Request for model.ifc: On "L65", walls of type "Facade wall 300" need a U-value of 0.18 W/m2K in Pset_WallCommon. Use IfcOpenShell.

First a look at what the model holds.

```python
import ifcopenshell
import ifcopenshell.util.element

model = ifcopenshell.open("model.ifc")
print(model.schema)
storey = next(s for s in model.by_type("IfcBuildingStorey") if s.Name == "L65")
walls = [e for e in ifcopenshell.util.element.get_decomposition(storey) if e.is_a("IfcWall")]
seen = {}
for e in walls:
    element_type = ifcopenshell.util.element.get_type(e)
    key = (element_type.Name if element_type != e and element_type else None, ifcopenshell.util.element.get_pset(e, "Pset_WallCommon", "ThermalTransmittance"))
    seen[key] = seen.get(key, 0) + 1
for (name, value), count in sorted(seen.items(), key=str):
    print(count, "x", name, "|", value)
```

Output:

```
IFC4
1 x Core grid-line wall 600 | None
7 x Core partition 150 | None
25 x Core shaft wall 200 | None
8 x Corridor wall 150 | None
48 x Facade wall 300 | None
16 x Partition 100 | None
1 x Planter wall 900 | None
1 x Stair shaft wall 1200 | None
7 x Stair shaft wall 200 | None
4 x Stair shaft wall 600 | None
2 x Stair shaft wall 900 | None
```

```python
import ifcopenshell
import ifcopenshell.api.pset
import ifcopenshell.util.element

model = ifcopenshell.open("model.ifc")

storey = next(s for s in model.by_type("IfcBuildingStorey") if s.Name == "L65")
walls = [e for e in ifcopenshell.util.element.get_decomposition(storey) if e.is_a("IfcWall")]

count = 0
for e in walls:
    element_type = ifcopenshell.util.element.get_type(e)
    if element_type in (None, e) or element_type.Name != "Facade wall 300":
        continue
    # add_pset returns the element's existing set when there is one.
    pset = ifcopenshell.api.pset.add_pset(model, product=e, name="Pset_WallCommon")
    ifcopenshell.api.pset.edit_pset(model, pset=pset, properties={"ThermalTransmittance": 0.18})
    count += 1

print(count, "walls updated")

model.write("model_v2.ifc")
```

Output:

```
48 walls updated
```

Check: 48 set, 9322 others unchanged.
